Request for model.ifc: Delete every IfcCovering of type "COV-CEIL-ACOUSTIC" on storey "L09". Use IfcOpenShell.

First a look at what the model holds.

```python
import ifcopenshell
import ifcopenshell.util.element

model = ifcopenshell.open("model.ifc")
print(model.schema)
storey = next(s for s in model.by_type("IfcBuildingStorey") if s.Name == "L09")
coverings = [e for e in ifcopenshell.util.element.get_decomposition(storey) if e.is_a("IfcCovering")]
seen = {}
for e in coverings:
    element_type = ifcopenshell.util.element.get_type(e)
    name = element_type.Name if element_type not in (None, e) else None
    seen[name] = seen.get(name, 0) + 1
for name, count in sorted(seen.items(), key=str):
    print(count, "x", name)
```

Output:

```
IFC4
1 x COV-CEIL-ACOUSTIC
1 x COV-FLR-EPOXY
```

```python
import ifcopenshell
import ifcopenshell.api.root
import ifcopenshell.util.element

model = ifcopenshell.open("model.ifc")

storey = next(s for s in model.by_type("IfcBuildingStorey") if s.Name == "L09")
coverings = [e for e in ifcopenshell.util.element.get_decomposition(storey) if e.is_a("IfcCovering")]
targets = [e for e in coverings if (t := ifcopenshell.util.element.get_type(e)) not in (None, e) and t.Name == "COV-CEIL-ACOUSTIC"]

for e in targets:
    ifcopenshell.api.root.remove_product(model, product=e)
print(len(targets), "removed")

model.write("model_edited.ifc")
```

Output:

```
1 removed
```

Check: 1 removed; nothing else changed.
